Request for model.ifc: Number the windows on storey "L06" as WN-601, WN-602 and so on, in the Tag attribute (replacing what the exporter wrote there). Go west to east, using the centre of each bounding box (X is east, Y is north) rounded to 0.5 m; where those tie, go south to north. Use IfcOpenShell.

First a look at what the model holds.

```python
import ifcopenshell
import ifcopenshell.util.element
import ifcopenshell.util.placement

model = ifcopenshell.open("model.ifc")
print(model.schema)
storey = next(s for s in model.by_type("IfcBuildingStorey") if s.Name == "L06")
windows = [e for e in ifcopenshell.util.element.get_decomposition(storey) if e.is_a("IfcWindow")]
for e in sorted(windows, key=lambda e: e.id()):
    origin = ifcopenshell.util.placement.get_local_placement(e.ObjectPlacement)[:3, 3]
    print(e.id(), e.Tag, e.Name, origin.round(2) + 0.0, sep=" | ")
```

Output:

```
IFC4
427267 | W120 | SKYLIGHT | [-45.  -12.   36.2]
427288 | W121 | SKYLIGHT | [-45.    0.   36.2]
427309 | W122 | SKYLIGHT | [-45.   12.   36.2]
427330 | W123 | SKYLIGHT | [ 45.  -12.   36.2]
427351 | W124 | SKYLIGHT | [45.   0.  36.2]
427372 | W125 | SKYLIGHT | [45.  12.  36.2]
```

```python
import ifcopenshell
import ifcopenshell.geom
import ifcopenshell.util.element
import ifcopenshell.util.shape

model = ifcopenshell.open("model.ifc")
settings = ifcopenshell.geom.settings()
settings.set("use-world-coords", True)


def centre(element):
    shape = ifcopenshell.geom.create_shape(settings, element)
    return ifcopenshell.util.shape.get_bbox_centroid(shape.geometry)


storey = next(s for s in model.by_type("IfcBuildingStorey") if s.Name == "L06")
windows = [e for e in ifcopenshell.util.element.get_decomposition(storey) if e.is_a("IfcWindow")]

# Insertion points can sit at a corner or the storey origin, so sort by the geometry (in metres).
centres = {e: centre(e) for e in windows}
windows.sort(key=lambda e: (round(centres[e][0] / 0.5), centres[e][1]))

for i, e in enumerate(windows, start=1):
    number = f"WN-6{i:02d}"
    e.Tag = number
    print(e.id(), number)

model.write("model_edited.ifc")
```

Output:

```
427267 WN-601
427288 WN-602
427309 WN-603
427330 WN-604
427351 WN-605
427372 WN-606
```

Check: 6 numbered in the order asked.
